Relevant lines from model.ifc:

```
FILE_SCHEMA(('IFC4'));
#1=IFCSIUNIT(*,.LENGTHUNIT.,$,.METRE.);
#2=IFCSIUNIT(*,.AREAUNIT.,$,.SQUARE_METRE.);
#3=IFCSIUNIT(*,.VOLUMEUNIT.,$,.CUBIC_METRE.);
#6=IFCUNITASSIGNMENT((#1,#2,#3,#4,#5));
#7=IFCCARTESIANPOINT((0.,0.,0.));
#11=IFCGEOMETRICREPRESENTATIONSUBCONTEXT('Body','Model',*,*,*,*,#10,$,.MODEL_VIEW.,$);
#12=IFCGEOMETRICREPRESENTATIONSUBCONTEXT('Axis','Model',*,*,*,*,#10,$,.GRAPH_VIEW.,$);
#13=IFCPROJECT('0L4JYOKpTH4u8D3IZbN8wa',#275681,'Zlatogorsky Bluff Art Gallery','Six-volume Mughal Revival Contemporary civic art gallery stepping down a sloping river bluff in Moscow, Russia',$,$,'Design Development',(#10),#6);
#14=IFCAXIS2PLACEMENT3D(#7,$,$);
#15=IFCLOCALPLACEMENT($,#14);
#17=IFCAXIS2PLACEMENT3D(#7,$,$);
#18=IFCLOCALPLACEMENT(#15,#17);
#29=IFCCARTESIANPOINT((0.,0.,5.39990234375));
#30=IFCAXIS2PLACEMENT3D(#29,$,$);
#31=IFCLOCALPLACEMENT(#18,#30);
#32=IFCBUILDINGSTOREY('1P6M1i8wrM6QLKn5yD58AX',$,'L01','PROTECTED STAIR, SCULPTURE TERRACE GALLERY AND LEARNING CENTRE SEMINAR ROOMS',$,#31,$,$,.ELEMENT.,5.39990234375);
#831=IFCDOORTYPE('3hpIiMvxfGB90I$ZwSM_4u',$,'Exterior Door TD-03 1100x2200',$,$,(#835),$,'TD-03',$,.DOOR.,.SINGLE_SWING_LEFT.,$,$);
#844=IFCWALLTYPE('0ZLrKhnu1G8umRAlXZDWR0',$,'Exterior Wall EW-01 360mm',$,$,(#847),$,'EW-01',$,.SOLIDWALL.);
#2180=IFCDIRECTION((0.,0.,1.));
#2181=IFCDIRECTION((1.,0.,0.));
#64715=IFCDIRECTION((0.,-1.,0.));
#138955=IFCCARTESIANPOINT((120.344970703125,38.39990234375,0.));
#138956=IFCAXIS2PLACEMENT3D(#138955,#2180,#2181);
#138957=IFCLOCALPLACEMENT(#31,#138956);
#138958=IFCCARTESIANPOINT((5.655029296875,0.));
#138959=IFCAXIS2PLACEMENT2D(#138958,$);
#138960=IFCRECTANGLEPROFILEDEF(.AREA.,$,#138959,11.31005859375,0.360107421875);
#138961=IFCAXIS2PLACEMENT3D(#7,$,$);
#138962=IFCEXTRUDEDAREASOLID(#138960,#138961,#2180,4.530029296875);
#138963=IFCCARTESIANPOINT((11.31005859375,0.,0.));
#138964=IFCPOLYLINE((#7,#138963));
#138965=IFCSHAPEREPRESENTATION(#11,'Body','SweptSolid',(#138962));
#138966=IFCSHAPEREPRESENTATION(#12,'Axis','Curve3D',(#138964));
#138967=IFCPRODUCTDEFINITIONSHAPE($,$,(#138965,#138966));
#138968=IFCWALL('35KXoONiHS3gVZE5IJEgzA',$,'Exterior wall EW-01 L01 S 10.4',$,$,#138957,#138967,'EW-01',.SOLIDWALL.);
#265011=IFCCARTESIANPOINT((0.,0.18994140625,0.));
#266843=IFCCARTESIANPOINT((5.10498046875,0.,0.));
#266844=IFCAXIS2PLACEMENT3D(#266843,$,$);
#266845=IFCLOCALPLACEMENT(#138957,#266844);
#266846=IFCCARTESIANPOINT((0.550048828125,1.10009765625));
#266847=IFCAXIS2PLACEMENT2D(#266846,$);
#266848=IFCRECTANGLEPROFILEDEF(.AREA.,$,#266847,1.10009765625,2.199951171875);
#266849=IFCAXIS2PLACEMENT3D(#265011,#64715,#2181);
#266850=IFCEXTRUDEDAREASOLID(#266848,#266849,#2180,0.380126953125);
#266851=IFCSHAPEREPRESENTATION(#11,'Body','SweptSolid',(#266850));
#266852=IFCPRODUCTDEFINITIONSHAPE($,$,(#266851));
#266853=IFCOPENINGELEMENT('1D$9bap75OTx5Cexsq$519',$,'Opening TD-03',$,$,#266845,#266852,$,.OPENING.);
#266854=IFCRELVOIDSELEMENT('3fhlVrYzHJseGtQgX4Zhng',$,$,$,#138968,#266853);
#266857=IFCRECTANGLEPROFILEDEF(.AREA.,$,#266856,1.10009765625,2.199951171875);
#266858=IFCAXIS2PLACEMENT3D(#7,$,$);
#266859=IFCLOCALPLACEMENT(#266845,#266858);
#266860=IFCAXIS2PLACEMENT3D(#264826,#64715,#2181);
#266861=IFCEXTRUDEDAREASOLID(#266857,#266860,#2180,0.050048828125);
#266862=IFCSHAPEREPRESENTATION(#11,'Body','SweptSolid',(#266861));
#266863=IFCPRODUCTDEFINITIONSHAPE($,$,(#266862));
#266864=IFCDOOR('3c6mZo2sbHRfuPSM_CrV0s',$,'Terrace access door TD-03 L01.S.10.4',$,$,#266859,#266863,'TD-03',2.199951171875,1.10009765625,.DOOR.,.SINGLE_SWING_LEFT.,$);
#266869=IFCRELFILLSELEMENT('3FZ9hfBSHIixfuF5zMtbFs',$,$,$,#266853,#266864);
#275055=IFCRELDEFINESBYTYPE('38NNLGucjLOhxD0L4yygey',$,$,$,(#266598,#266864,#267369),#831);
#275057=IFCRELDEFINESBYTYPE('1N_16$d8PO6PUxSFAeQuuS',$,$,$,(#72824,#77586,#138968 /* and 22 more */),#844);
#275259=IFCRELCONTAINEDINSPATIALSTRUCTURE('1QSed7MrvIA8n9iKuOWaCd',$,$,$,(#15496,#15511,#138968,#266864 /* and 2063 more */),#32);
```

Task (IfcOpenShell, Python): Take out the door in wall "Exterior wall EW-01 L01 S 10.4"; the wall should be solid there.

```python
import ifcopenshell
import ifcopenshell.api.feature
import ifcopenshell.api.root
import ifcopenshell.geom
import ifcopenshell.util.shape

model = ifcopenshell.open("model.ifc")
settings = ifcopenshell.geom.settings()


def volume(element):
    """Net volume in cubic metres, openings subtracted."""
    shape = ifcopenshell.geom.create_shape(settings, element)
    return ifcopenshell.util.shape.get_volume(shape.geometry)


door = model.by_guid("3c6mZo2sbHRfuPSM_CrV0s")
opening = door.FillsVoids[0].RelatingOpeningElement
wall = opening.VoidsElements[0].RelatingBuildingElement
before = volume(wall)

ifcopenshell.api.root.remove_product(model, product=door)
ifcopenshell.api.feature.remove_feature(model, feature=opening)

after = volume(wall)

print(f"wall volume {before:.3f} -> {after:.3f} m3")

model.write("model_updated.ifc")
```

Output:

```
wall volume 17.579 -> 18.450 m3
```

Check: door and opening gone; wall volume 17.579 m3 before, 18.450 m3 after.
